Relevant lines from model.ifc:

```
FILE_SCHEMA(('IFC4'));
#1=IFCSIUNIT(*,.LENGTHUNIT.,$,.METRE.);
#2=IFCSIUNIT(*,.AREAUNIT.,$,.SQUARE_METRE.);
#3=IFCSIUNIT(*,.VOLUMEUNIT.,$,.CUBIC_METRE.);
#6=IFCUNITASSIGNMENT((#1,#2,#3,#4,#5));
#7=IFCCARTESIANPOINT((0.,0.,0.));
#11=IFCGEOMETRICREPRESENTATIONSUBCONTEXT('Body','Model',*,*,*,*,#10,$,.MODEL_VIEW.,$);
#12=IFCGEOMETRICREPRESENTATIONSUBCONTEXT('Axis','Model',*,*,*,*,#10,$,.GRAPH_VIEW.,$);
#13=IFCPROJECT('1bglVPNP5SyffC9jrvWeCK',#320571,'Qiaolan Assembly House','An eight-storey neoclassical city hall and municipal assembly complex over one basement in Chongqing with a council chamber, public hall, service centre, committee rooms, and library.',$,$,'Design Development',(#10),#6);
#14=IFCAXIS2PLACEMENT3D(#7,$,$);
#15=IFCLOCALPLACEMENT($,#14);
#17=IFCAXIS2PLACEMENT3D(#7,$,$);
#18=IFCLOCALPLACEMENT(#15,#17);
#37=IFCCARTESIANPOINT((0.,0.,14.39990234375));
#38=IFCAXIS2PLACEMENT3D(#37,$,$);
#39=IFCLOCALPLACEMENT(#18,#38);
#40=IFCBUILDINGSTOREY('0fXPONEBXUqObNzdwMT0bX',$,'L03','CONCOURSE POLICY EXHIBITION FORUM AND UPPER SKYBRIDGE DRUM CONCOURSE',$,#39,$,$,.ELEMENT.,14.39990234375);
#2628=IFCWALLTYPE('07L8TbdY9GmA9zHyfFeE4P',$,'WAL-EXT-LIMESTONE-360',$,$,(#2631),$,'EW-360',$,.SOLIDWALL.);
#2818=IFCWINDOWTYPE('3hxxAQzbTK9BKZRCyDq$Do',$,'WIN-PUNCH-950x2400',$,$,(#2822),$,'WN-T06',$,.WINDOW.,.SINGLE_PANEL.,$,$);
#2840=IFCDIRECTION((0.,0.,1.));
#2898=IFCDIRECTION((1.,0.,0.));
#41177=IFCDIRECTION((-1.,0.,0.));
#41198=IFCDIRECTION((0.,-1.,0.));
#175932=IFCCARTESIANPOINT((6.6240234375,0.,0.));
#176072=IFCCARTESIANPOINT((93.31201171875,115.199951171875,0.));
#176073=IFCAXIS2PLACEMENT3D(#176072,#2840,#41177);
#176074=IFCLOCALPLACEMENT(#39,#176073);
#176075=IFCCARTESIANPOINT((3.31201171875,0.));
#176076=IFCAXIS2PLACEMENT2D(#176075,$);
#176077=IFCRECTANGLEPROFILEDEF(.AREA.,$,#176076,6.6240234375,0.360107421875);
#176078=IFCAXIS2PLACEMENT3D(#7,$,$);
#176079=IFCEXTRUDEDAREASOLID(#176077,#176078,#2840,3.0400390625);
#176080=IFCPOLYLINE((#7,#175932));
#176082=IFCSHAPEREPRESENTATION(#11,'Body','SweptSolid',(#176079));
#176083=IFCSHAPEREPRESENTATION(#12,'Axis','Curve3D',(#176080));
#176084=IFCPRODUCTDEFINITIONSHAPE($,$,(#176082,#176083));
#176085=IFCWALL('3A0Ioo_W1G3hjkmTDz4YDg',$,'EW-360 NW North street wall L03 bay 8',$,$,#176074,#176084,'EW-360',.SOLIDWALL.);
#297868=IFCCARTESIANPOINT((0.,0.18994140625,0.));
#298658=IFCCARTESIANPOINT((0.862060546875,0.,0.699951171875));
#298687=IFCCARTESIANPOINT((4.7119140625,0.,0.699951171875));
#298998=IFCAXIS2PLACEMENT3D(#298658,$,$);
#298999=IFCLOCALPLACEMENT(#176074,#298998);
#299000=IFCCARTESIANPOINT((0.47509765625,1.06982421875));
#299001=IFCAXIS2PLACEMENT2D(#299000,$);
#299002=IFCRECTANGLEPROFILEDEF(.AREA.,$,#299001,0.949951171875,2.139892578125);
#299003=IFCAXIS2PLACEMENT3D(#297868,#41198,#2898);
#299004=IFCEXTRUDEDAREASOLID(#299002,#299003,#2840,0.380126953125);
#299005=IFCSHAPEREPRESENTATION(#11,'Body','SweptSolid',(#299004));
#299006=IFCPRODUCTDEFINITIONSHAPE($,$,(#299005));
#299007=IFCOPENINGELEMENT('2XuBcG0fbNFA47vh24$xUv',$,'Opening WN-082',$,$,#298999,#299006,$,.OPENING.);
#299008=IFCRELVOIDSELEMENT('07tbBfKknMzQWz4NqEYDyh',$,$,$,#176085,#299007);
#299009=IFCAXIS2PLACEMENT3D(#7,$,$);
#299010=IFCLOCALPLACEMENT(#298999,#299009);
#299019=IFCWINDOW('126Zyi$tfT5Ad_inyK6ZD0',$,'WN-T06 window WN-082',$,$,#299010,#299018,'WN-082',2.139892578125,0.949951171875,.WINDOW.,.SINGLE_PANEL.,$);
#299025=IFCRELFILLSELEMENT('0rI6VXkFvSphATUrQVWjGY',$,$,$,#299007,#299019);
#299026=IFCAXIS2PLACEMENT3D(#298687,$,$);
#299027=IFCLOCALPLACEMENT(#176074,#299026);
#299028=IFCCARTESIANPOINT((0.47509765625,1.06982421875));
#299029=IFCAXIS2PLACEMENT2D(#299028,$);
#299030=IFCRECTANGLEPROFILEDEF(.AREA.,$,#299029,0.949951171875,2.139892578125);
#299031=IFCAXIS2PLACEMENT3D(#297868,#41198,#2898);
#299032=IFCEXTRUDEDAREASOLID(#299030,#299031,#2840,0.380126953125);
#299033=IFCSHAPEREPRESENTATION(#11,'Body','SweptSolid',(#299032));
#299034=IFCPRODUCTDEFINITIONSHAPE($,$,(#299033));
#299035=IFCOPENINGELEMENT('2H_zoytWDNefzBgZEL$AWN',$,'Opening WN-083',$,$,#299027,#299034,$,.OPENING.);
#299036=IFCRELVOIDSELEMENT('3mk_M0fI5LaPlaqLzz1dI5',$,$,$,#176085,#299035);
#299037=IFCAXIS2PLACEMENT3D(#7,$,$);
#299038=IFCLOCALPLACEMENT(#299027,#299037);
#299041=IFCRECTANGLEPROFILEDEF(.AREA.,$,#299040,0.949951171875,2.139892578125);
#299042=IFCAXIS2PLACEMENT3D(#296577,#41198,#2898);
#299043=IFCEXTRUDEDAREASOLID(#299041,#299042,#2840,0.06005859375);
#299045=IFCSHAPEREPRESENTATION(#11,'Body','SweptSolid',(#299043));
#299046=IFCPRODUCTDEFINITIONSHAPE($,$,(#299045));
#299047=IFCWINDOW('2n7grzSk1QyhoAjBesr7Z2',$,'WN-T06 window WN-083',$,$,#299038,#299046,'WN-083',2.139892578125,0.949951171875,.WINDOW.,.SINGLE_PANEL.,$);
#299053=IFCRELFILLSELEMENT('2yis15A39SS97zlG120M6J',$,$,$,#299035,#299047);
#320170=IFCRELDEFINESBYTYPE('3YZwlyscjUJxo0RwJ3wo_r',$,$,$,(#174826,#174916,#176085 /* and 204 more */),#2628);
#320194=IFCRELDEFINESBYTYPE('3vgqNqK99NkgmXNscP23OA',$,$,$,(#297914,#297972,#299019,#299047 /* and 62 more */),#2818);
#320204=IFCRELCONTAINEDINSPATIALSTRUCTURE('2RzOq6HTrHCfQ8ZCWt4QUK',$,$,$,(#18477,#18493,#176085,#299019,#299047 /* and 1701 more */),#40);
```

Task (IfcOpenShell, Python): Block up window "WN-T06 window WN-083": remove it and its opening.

```python
import ifcopenshell
import ifcopenshell.api.feature
import ifcopenshell.api.root
import ifcopenshell.geom
import ifcopenshell.util.shape

model = ifcopenshell.open("model.ifc")
settings = ifcopenshell.geom.settings()


def volume(element):
    """Net volume in cubic metres, openings subtracted."""
    shape = ifcopenshell.geom.create_shape(settings, element)
    return ifcopenshell.util.shape.get_volume(shape.geometry)


window = model.by_id(299047)
opening = window.FillsVoids[0].RelatingOpeningElement
wall = opening.VoidsElements[0].RelatingBuildingElement
before = volume(wall)

ifcopenshell.api.root.remove_product(model, product=window)
ifcopenshell.api.feature.remove_feature(model, feature=opening)

after = volume(wall)

print(f"wall volume {before:.3f} -> {after:.3f} m3")

model.write("model-out.ifc")
```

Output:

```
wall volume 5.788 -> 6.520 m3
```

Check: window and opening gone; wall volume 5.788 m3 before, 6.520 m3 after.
